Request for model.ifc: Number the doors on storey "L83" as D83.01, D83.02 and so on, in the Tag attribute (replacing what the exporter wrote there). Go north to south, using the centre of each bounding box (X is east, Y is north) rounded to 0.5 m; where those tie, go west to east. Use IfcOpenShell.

First a look at what the model holds.

```python
import ifcopenshell
import ifcopenshell.util.element
import ifcopenshell.util.placement

model = ifcopenshell.open("model.ifc")
print(model.schema)
storey = next(s for s in model.by_type("IfcBuildingStorey") if s.Name == "L83")
doors = [e for e in ifcopenshell.util.element.get_decomposition(storey) if e.is_a("IfcDoor")]
for e in sorted(doors, key=lambda e: e.id()):
    origin = ifcopenshell.util.placement.get_local_placement(e.ObjectPlacement)[:3, 3]
    print(e.id(), e.Tag, e.Name, origin.round(2) + 0.0, sep=" | ")
```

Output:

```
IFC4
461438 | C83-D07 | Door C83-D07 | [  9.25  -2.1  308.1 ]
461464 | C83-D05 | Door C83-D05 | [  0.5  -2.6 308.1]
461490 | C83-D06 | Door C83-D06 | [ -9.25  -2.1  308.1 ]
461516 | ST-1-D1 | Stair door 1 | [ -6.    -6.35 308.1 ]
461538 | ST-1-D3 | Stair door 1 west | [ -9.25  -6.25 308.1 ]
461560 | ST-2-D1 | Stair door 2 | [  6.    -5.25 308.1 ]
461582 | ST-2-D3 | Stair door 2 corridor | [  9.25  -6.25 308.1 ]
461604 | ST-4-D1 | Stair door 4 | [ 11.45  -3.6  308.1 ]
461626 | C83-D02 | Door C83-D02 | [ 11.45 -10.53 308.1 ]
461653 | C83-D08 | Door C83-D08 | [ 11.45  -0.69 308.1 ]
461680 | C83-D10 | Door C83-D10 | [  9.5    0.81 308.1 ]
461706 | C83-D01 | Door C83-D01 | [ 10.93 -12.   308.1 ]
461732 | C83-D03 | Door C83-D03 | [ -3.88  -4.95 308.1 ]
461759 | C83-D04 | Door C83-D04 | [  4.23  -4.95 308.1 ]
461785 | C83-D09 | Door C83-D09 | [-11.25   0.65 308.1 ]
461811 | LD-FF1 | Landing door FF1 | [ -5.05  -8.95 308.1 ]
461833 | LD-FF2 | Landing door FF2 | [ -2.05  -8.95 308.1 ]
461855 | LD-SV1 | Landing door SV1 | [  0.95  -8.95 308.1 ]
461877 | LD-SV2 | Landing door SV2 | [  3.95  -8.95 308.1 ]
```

```python
import ifcopenshell
import ifcopenshell.geom
import ifcopenshell.util.element
import ifcopenshell.util.shape

model = ifcopenshell.open("model.ifc")
settings = ifcopenshell.geom.settings()
settings.set("use-world-coords", True)


def centre(element):
    shape = ifcopenshell.geom.create_shape(settings, element)
    return ifcopenshell.util.shape.get_bbox_centroid(shape.geometry)


storey = next(s for s in model.by_type("IfcBuildingStorey") if s.Name == "L83")
doors = [e for e in ifcopenshell.util.element.get_decomposition(storey) if e.is_a("IfcDoor")]

# Insertion points can sit at a corner or the storey origin, so sort by the geometry (in metres).
centres = {e: centre(e) for e in doors}
doors.sort(key=lambda e: (-round(centres[e][1] / 0.5), centres[e][0]))

for i, e in enumerate(doors, start=1):
    number = f"D83.{i:02d}"
    e.Tag = number
    print(e.id(), number)

model.write("model-out.ifc")
```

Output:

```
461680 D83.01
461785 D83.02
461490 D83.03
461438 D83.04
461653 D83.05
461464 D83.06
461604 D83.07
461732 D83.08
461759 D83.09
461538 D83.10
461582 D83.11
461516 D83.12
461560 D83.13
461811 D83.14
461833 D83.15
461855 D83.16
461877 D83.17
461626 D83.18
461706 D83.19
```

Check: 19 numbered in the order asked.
